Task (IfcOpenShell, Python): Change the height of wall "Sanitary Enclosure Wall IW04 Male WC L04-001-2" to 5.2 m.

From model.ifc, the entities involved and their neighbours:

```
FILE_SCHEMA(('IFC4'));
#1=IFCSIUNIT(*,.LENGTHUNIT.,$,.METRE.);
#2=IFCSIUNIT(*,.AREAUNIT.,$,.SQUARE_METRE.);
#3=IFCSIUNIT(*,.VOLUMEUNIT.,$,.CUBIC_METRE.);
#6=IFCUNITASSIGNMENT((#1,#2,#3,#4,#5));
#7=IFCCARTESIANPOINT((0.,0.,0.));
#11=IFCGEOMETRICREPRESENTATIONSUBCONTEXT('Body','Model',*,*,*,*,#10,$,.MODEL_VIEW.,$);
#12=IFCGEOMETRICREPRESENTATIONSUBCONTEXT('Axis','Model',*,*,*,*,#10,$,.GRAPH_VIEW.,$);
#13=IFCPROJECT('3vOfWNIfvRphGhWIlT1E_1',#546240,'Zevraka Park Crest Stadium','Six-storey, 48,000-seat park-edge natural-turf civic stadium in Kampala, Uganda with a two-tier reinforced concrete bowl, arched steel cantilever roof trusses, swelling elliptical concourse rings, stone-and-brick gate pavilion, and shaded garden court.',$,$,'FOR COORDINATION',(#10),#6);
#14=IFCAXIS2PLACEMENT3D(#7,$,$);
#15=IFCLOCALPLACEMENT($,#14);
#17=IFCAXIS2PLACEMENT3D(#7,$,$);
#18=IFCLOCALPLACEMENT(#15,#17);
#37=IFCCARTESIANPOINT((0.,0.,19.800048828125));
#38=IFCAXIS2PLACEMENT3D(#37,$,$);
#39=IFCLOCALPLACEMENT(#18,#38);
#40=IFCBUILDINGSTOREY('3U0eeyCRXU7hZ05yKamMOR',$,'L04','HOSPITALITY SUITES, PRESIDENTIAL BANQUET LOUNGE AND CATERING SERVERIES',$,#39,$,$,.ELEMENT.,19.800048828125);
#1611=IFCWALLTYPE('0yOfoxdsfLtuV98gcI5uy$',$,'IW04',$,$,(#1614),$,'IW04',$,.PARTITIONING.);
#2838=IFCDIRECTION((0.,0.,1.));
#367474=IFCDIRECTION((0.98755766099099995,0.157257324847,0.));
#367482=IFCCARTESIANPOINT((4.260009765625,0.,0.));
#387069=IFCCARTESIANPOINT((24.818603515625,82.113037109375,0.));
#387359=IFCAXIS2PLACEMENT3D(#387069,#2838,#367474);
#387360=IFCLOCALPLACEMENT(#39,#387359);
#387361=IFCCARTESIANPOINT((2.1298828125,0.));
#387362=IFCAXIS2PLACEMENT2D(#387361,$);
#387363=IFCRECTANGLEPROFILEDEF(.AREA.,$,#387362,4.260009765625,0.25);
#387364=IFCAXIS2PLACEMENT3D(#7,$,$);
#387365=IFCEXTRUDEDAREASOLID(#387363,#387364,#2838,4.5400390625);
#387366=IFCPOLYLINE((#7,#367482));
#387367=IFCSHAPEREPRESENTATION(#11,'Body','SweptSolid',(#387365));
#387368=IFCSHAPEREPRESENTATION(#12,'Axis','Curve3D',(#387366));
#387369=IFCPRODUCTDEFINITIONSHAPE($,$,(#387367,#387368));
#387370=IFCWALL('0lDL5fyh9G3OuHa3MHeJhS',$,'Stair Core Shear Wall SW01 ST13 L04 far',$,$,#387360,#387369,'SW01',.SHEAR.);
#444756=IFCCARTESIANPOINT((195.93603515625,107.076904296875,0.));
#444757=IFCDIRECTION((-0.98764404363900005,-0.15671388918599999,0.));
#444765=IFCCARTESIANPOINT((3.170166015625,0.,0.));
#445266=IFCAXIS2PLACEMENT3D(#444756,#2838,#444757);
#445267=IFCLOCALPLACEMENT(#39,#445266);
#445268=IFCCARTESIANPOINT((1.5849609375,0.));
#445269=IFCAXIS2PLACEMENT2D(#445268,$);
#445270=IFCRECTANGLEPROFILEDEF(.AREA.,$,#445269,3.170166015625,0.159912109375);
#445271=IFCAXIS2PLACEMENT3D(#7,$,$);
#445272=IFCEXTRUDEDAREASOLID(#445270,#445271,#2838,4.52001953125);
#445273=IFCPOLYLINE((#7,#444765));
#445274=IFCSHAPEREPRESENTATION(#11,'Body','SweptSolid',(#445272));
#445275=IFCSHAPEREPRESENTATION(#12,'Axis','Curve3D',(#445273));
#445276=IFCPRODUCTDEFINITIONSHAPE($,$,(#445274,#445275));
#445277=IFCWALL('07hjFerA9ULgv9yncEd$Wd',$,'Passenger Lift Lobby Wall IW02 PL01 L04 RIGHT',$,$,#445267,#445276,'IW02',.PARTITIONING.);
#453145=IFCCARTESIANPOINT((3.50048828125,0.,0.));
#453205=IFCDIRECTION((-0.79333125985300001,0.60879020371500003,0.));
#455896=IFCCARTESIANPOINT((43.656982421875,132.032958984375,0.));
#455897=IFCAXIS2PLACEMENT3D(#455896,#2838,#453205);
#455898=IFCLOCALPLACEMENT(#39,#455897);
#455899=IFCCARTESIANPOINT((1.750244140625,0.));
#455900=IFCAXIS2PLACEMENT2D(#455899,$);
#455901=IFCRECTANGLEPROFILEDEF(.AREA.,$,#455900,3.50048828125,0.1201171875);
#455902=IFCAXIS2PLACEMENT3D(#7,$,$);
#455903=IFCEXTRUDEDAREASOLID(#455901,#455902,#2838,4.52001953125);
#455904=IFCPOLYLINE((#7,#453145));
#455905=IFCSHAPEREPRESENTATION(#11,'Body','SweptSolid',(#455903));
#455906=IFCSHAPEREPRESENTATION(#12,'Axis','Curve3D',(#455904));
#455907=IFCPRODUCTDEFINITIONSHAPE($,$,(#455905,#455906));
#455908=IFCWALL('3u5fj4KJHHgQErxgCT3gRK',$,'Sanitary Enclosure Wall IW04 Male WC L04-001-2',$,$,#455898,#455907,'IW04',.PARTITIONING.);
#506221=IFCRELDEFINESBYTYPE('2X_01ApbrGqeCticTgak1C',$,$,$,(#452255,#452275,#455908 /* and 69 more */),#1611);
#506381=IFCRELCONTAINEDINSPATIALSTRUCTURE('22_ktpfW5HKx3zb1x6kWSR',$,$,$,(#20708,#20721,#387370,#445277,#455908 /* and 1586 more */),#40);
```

```python
import ifcopenshell
import ifcopenshell.geom
import ifcopenshell.util.representation
import ifcopenshell.util.shape
import ifcopenshell.util.unit

model = ifcopenshell.open("model.ifc")
unit_scale = ifcopenshell.util.unit.calculate_unit_scale(model)
settings = ifcopenshell.geom.settings()


def volume(element):
    """Net volume in cubic metres, openings subtracted."""
    shape = ifcopenshell.geom.create_shape(settings, element)
    return ifcopenshell.util.shape.get_volume(shape.geometry)


wall = model.by_guid("3u5fj4KJHHgQErxgCT3gRK")
before = volume(wall)

body = ifcopenshell.util.representation.get_representation(wall, "Model", "Body")
solid = body.Items[0]
old_height = solid.Depth
solid.Depth = 5.2 / unit_scale
after = volume(wall)

print(f"height {old_height:g} -> {solid.Depth:g}, volume {before:.3f} -> {after:.3f} m3")

model.write("model-out.ifc")
```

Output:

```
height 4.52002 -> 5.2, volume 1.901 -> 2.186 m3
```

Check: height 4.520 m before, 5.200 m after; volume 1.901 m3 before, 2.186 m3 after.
